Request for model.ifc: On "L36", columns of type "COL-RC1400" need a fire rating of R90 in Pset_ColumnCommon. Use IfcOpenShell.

First a look at what the model holds.

```python
import ifcopenshell
import ifcopenshell.util.element

model = ifcopenshell.open("model.ifc")
print(model.schema)
storey = next(s for s in model.by_type("IfcBuildingStorey") if s.Name == "L36")
columns = [e for e in ifcopenshell.util.element.get_decomposition(storey) if e.is_a("IfcColumn")]
seen = {}
for e in columns:
    element_type = ifcopenshell.util.element.get_type(e)
    key = (element_type.Name if element_type != e and element_type else None, ifcopenshell.util.element.get_pset(e, "Pset_ColumnCommon", "FireRating"))
    seen[key] = seen.get(key, 0) + 1
for (name, value), count in sorted(seen.items(), key=str):
    print(count, "x", name, "|", value)
```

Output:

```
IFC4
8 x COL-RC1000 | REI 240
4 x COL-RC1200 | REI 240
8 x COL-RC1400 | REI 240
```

```python
import ifcopenshell
import ifcopenshell.api.pset
import ifcopenshell.util.element

model = ifcopenshell.open("model.ifc")

storey = next(s for s in model.by_type("IfcBuildingStorey") if s.Name == "L36")
columns = [e for e in ifcopenshell.util.element.get_decomposition(storey) if e.is_a("IfcColumn")]

count = 0
for e in columns:
    element_type = ifcopenshell.util.element.get_type(e)
    if element_type in (None, e) or element_type.Name != "COL-RC1400":
        continue
    found = ifcopenshell.util.element.get_pset(e, "Pset_ColumnCommon", should_inherit=False)
    if found:
        pset = model.by_id(found["id"])
        if len(ifcopenshell.util.element.get_elements_by_pset(pset)) > 1:
            pset = ifcopenshell.api.pset.unshare_pset(model, products=[e], pset=pset)[0]
    else:
        pset = ifcopenshell.api.pset.add_pset(model, product=e, name="Pset_ColumnCommon")
    ifcopenshell.api.pset.edit_pset(model, pset=pset, properties={"FireRating": "R90"})
    count += 1

print(count, "columns updated")

model.write("model_edited.ifc")
```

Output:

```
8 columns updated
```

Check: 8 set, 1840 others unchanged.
